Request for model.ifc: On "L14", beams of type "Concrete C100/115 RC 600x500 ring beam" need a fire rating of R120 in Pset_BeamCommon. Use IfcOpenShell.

First a look at what the model holds.

```python
import ifcopenshell
import ifcopenshell.util.element

model = ifcopenshell.open("model.ifc")
print(model.schema)
storey = next(s for s in model.by_type("IfcBuildingStorey") if s.Name == "L14")
beams = [e for e in ifcopenshell.util.element.get_decomposition(storey) if e.is_a("IfcBeam")]
seen = {}
for e in beams:
    element_type = ifcopenshell.util.element.get_type(e)
    key = (element_type.Name if element_type != e and element_type else None, ifcopenshell.util.element.get_pset(e, "Pset_BeamCommon", "FireRating"))
    seen[key] = seen.get(key, 0) + 1
for (name, value), count in sorted(seen.items(), key=str):
    print(count, "x", name, "|", value)
```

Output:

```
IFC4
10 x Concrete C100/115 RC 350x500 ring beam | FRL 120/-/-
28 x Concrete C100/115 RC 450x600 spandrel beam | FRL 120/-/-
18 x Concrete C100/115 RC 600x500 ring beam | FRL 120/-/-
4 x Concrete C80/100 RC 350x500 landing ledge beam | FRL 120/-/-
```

```python
import ifcopenshell
import ifcopenshell.api.pset
import ifcopenshell.util.element

model = ifcopenshell.open("model.ifc")

storey = next(s for s in model.by_type("IfcBuildingStorey") if s.Name == "L14")
beams = [e for e in ifcopenshell.util.element.get_decomposition(storey) if e.is_a("IfcBeam")]

count = 0
for e in beams:
    element_type = ifcopenshell.util.element.get_type(e)
    if element_type in (None, e) or element_type.Name != "Concrete C100/115 RC 600x500 ring beam":
        continue
    found = ifcopenshell.util.element.get_pset(e, "Pset_BeamCommon", should_inherit=False)
    if found:
        pset = model.by_id(found["id"])
        if len(ifcopenshell.util.element.get_elements_by_pset(pset)) > 1:
            pset = ifcopenshell.api.pset.unshare_pset(model, products=[e], pset=pset)[0]
    else:
        pset = ifcopenshell.api.pset.add_pset(model, product=e, name="Pset_BeamCommon")
    ifcopenshell.api.pset.edit_pset(model, pset=pset, properties={"FireRating": "R120"})
    count += 1

print(count, "beams updated")

model.write("model_edited.ifc")
```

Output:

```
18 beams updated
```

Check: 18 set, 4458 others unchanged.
